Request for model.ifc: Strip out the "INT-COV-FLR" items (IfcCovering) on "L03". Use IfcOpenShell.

First a look at what the model holds.

```python
import ifcopenshell
import ifcopenshell.util.element

model = ifcopenshell.open("model.ifc")
print(model.schema)
storey = next(s for s in model.by_type("IfcBuildingStorey") if s.Name == "L03")
coverings = [e for e in ifcopenshell.util.element.get_decomposition(storey) if e.is_a("IfcCovering")]
seen = {}
for e in coverings:
    element_type = ifcopenshell.util.element.get_type(e)
    name = element_type.Name if element_type not in (None, e) else None
    seen[name] = seen.get(name, 0) + 1
for name, count in sorted(seen.items(), key=str):
    print(count, "x", name)
```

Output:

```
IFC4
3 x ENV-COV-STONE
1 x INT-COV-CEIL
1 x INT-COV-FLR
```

```python
import ifcopenshell
import ifcopenshell.api.root
import ifcopenshell.util.element

model = ifcopenshell.open("model.ifc")

storey = next(s for s in model.by_type("IfcBuildingStorey") if s.Name == "L03")
coverings = [e for e in ifcopenshell.util.element.get_decomposition(storey) if e.is_a("IfcCovering")]
targets = [e for e in coverings if (t := ifcopenshell.util.element.get_type(e)) not in (None, e) and t.Name == "INT-COV-FLR"]

for e in targets:
    ifcopenshell.api.root.remove_product(model, product=e)
print(len(targets), "removed")

model.write("model_v2.ifc")
```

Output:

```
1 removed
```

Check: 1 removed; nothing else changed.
